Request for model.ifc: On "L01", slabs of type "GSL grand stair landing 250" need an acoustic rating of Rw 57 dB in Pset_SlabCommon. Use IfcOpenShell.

First a look at what the model holds.

```python
import ifcopenshell
import ifcopenshell.util.element

model = ifcopenshell.open("model.ifc")
print(model.schema)
storey = next(s for s in model.by_type("IfcBuildingStorey") if s.Name == "L01")
slabs = [e for e in ifcopenshell.util.element.get_decomposition(storey) if e.is_a("IfcSlab")]
seen = {}
for e in slabs:
    element_type = ifcopenshell.util.element.get_type(e)
    key = (element_type.Name if element_type != e and element_type else None, ifcopenshell.util.element.get_pset(e, "Pset_SlabCommon", "AcousticRating"))
    seen[key] = seen.get(key, 0) + 1
for (name, value), count in sorted(seen.items(), key=str):
    print(count, "x", name, "|", value)
```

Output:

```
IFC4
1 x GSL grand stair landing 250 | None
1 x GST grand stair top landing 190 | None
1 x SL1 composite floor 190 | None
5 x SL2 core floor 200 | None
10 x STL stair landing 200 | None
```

```python
import ifcopenshell
import ifcopenshell.api.pset
import ifcopenshell.util.element

model = ifcopenshell.open("model.ifc")

storey = next(s for s in model.by_type("IfcBuildingStorey") if s.Name == "L01")
slabs = [e for e in ifcopenshell.util.element.get_decomposition(storey) if e.is_a("IfcSlab")]

count = 0
for e in slabs:
    element_type = ifcopenshell.util.element.get_type(e)
    if element_type in (None, e) or element_type.Name != "GSL grand stair landing 250":
        continue
    found = ifcopenshell.util.element.get_pset(e, "Pset_SlabCommon", should_inherit=False)
    if found:
        pset = model.by_id(found["id"])
        if len(ifcopenshell.util.element.get_elements_by_pset(pset)) > 1:
            pset = ifcopenshell.api.pset.unshare_pset(model, products=[e], pset=pset)[0]
    else:
        pset = ifcopenshell.api.pset.add_pset(model, product=e, name="Pset_SlabCommon")
    ifcopenshell.api.pset.edit_pset(model, pset=pset, properties={"AcousticRating": "Rw 57 dB"})
    count += 1

print(count, "slabs updated")

model.write("model_updated.ifc")
```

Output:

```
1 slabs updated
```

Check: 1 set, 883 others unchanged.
